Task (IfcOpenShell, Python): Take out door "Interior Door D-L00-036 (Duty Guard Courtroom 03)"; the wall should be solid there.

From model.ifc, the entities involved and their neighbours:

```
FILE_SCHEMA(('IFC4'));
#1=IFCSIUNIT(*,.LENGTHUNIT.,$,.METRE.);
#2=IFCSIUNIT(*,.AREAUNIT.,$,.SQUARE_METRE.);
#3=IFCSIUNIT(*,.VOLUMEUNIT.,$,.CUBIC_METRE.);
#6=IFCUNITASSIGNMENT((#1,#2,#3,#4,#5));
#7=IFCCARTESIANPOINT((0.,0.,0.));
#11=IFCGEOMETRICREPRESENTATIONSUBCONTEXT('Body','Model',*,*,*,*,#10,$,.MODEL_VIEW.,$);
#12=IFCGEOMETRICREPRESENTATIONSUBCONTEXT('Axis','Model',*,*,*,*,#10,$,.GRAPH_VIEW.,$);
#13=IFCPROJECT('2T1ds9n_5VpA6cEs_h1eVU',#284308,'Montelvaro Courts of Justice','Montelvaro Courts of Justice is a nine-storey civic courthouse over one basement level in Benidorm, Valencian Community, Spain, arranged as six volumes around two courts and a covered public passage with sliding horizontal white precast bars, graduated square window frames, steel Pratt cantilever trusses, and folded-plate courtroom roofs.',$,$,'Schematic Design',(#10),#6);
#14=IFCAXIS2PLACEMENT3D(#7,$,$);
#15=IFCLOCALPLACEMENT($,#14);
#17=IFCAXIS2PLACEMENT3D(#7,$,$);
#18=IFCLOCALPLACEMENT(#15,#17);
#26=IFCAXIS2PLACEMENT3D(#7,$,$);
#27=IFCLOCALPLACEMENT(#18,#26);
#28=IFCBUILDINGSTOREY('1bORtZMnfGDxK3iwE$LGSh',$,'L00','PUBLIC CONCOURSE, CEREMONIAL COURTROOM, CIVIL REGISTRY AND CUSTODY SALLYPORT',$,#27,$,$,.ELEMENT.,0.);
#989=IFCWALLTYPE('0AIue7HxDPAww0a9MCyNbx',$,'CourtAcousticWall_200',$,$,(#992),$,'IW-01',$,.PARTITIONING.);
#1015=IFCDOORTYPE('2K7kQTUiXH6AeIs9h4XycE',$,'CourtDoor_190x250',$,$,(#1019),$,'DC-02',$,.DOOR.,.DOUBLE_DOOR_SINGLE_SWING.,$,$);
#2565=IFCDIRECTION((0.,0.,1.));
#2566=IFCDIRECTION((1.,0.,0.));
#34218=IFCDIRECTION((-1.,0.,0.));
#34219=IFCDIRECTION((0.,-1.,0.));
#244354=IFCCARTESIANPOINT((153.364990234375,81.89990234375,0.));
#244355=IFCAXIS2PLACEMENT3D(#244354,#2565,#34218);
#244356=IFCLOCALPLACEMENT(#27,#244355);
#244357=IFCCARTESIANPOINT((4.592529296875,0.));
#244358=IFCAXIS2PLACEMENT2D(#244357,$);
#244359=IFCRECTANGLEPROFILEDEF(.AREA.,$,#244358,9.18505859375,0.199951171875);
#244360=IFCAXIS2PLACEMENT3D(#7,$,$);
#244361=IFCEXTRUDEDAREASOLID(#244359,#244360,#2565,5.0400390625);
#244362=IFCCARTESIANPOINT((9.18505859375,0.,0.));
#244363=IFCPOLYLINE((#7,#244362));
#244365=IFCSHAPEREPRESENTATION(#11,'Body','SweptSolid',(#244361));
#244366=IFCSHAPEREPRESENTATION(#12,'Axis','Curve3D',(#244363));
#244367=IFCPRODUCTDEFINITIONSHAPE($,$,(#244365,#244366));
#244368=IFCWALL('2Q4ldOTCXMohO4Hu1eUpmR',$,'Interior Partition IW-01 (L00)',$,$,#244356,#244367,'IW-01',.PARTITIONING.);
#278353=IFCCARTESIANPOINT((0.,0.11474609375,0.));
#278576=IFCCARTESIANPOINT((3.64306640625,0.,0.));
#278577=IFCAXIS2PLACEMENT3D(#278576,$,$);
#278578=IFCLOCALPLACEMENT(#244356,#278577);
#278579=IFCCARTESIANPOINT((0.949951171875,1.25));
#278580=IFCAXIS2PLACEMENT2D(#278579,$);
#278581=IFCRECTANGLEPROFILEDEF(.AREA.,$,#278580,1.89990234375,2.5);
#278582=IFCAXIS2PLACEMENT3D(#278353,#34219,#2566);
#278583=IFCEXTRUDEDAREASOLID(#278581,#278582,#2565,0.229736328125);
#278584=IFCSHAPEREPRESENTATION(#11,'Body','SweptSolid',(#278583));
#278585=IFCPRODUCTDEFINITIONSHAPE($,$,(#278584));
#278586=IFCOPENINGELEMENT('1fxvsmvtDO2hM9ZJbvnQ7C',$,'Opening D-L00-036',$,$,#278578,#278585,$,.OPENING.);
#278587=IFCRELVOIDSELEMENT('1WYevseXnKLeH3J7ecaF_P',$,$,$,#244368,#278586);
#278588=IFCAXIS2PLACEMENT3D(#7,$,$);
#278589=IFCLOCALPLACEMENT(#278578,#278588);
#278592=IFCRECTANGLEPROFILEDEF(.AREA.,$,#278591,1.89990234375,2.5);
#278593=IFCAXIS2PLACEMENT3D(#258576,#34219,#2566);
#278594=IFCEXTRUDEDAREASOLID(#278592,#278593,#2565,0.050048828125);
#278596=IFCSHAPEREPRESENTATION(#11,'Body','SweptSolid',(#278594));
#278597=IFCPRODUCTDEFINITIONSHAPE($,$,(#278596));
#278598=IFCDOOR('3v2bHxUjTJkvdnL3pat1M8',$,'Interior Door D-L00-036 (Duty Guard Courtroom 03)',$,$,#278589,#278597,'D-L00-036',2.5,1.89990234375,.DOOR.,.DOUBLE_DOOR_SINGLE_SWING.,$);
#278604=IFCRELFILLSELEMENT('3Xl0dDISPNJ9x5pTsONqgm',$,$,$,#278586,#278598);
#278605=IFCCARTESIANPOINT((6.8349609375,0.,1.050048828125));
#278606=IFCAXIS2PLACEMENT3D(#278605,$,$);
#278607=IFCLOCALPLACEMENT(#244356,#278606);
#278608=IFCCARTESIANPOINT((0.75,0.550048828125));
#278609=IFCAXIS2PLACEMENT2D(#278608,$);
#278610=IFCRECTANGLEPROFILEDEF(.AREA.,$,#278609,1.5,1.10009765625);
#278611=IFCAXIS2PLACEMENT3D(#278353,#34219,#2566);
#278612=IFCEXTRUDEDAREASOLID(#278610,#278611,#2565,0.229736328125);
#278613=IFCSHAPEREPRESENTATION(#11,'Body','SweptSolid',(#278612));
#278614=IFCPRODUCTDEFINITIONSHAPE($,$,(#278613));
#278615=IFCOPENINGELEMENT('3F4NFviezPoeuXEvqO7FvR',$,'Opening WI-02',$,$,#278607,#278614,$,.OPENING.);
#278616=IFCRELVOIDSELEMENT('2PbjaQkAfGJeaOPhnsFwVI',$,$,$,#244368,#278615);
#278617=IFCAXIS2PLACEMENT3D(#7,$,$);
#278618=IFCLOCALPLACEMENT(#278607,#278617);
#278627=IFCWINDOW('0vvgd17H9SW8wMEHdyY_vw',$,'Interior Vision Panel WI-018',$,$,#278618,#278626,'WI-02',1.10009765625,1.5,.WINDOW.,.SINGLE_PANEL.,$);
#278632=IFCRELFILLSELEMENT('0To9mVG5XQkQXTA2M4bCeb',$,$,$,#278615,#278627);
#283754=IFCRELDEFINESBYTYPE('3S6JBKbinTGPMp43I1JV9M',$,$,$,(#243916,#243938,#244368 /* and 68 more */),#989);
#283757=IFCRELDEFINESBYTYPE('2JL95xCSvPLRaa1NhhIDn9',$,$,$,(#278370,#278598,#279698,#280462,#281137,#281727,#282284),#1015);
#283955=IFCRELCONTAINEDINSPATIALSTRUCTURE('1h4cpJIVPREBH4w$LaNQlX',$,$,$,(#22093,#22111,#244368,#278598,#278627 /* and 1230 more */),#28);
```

```python
import ifcopenshell
import ifcopenshell.api.feature
import ifcopenshell.api.root
import ifcopenshell.geom
import ifcopenshell.util.shape

model = ifcopenshell.open("model.ifc")
settings = ifcopenshell.geom.settings()


def volume(element):
    """Net volume in cubic metres, openings subtracted."""
    shape = ifcopenshell.geom.create_shape(settings, element)
    return ifcopenshell.util.shape.get_volume(shape.geometry)


door = model.by_guid("3v2bHxUjTJkvdnL3pat1M8")
opening = door.FillsVoids[0].RelatingOpeningElement
wall = opening.VoidsElements[0].RelatingBuildingElement
before = volume(wall)

ifcopenshell.api.root.remove_product(model, product=door)
ifcopenshell.api.feature.remove_feature(model, feature=opening)

after = volume(wall)

print(f"wall volume {before:.3f} -> {after:.3f} m3")

model.write("model-out.ifc")
```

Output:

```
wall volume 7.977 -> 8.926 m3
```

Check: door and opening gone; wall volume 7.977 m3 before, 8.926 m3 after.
